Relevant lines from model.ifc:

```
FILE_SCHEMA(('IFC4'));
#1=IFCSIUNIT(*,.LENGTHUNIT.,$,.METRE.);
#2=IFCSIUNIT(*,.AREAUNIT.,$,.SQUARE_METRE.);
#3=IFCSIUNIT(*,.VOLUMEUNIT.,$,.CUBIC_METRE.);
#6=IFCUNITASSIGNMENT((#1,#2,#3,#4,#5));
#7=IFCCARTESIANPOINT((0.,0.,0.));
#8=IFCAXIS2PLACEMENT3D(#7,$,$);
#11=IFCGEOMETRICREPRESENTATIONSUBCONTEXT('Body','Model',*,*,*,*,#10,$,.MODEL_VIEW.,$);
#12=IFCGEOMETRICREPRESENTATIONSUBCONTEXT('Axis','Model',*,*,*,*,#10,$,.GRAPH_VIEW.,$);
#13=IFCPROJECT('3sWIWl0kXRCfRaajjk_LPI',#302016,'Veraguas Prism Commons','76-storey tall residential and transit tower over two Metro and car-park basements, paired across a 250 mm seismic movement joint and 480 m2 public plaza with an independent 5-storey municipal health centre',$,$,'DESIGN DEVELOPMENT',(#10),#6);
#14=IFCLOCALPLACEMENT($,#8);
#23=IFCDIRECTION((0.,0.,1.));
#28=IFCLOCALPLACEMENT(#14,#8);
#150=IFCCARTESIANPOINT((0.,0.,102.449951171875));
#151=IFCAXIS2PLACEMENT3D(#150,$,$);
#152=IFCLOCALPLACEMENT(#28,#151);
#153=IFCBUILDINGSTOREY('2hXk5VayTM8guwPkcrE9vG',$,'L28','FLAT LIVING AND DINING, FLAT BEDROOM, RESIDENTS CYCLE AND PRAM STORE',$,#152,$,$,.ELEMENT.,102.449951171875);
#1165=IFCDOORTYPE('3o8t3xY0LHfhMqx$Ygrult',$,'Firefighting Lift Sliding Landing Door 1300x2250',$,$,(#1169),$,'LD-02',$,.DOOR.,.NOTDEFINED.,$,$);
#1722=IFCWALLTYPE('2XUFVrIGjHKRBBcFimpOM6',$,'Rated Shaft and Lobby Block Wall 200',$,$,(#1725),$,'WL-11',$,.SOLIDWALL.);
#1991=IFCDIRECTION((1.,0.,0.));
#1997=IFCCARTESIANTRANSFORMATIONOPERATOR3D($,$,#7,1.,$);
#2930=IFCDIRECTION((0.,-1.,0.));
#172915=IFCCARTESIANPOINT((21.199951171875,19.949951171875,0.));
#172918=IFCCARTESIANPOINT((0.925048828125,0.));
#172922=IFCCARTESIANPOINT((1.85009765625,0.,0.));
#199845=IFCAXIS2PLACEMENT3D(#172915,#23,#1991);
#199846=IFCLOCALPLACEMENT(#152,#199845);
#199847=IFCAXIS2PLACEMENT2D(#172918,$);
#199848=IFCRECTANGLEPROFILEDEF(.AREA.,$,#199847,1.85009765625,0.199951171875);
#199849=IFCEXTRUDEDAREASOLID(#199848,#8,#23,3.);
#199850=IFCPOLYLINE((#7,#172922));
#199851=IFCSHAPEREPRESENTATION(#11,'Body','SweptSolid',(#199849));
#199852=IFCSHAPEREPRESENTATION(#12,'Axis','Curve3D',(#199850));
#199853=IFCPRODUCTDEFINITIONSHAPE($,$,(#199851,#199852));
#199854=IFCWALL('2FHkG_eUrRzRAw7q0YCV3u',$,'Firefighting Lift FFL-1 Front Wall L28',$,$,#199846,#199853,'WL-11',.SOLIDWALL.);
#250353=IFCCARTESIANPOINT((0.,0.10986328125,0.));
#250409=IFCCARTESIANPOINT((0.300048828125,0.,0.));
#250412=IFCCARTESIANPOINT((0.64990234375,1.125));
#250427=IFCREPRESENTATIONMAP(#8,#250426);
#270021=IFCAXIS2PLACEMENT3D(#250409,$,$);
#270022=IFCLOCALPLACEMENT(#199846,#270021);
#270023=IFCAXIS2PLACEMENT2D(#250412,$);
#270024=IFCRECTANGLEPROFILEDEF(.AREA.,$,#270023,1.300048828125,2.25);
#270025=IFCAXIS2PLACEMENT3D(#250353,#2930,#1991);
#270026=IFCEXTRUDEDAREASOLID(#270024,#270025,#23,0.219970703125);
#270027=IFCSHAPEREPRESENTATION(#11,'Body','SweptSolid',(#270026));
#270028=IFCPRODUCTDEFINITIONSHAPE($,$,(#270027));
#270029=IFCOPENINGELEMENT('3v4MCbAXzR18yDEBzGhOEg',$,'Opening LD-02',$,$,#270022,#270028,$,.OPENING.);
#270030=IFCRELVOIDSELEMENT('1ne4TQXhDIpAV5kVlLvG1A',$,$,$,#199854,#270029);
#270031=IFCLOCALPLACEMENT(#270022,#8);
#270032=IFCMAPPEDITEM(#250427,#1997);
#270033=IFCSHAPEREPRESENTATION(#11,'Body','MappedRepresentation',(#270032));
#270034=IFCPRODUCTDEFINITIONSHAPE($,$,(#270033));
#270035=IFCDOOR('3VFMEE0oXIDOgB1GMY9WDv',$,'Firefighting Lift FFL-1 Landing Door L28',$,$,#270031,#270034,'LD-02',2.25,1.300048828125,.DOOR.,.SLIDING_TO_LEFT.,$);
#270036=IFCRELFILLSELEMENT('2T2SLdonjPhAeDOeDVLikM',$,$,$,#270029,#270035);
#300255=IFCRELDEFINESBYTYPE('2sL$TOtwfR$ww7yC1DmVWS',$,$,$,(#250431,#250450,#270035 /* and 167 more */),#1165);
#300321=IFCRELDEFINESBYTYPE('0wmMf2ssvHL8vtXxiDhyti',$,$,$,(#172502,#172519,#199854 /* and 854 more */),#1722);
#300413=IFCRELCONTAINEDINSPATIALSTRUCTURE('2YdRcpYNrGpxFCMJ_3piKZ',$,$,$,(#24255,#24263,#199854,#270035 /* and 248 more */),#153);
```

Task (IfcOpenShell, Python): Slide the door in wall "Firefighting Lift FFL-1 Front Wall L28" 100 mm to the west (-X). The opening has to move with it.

```python
import ifcopenshell
import ifcopenshell.api.geometry
import ifcopenshell.util.placement
import ifcopenshell.util.unit

model = ifcopenshell.open("model.ifc")
unit_scale = ifcopenshell.util.unit.calculate_unit_scale(model)

door = model.by_id(270035)
opening = door.FillsVoids[0].RelatingOpeningElement
wall = opening.VoidsElements[0].RelatingBuildingElement

wall_matrix = ifcopenshell.util.placement.get_local_placement(wall.ObjectPlacement)
shift = wall_matrix[:3, 0] * -0.1 / unit_scale
before = ifcopenshell.util.placement.get_local_placement(door.ObjectPlacement)[:3, 3].copy()

# The door is placed relative to its opening, so it follows when the opening moves.
matrix = ifcopenshell.util.placement.get_local_placement(opening.ObjectPlacement)
matrix[:3, 3] += shift
ifcopenshell.api.geometry.edit_object_placement(
    model, product=opening, matrix=matrix, is_si=False, should_transform_children=True
)

after = ifcopenshell.util.placement.get_local_placement(door.ObjectPlacement)[:3, 3]
print("door moved by", (after - before).round(3) + 0.0)

model.write("model_rev.ifc")
```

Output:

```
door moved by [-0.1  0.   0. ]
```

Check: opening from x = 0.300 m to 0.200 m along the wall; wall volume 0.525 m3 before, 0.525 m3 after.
